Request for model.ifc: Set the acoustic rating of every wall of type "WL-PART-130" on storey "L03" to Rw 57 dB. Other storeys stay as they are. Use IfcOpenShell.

First a look at what the model holds.

```python
import ifcopenshell
import ifcopenshell.util.element

model = ifcopenshell.open("model.ifc")
print(model.schema)
storey = next(s for s in model.by_type("IfcBuildingStorey") if s.Name == "L03")
walls = [e for e in ifcopenshell.util.element.get_decomposition(storey) if e.is_a("IfcWall")]
seen = {}
for e in walls:
    element_type = ifcopenshell.util.element.get_type(e)
    key = (element_type.Name if element_type != e and element_type else None, ifcopenshell.util.element.get_pset(e, "Pset_WallCommon", "AcousticRating"))
    seen[key] = seen.get(key, 0) + 1
for (name, value), count in sorted(seen.items(), key=str):
    print(count, "x", name, "|", value)
```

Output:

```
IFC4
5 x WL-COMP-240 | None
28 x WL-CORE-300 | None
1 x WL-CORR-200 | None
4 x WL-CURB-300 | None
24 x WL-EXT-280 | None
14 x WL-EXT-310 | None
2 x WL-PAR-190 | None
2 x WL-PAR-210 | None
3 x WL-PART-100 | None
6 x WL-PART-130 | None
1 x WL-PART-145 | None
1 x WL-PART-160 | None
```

```python
import ifcopenshell
import ifcopenshell.api.pset
import ifcopenshell.util.element

model = ifcopenshell.open("model.ifc")

storey = next(s for s in model.by_type("IfcBuildingStorey") if s.Name == "L03")
walls = [e for e in ifcopenshell.util.element.get_decomposition(storey) if e.is_a("IfcWall")]

count = 0
for e in walls:
    element_type = ifcopenshell.util.element.get_type(e)
    if element_type in (None, e) or element_type.Name != "WL-PART-130":
        continue
    # add_pset returns the element's existing set when there is one.
    pset = ifcopenshell.api.pset.add_pset(model, product=e, name="Pset_WallCommon")
    ifcopenshell.api.pset.edit_pset(model, pset=pset, properties={"AcousticRating": "Rw 57 dB"})
    count += 1

print(count, "walls updated")

model.write("model_rev.ifc")
```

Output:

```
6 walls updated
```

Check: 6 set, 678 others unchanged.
